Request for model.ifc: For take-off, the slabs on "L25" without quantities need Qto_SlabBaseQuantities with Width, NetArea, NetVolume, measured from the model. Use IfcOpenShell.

First a look at what the model holds.

```python
import ifcopenshell
import ifcopenshell.util.element
import ifcopenshell.util.unit

model = ifcopenshell.open("model.ifc")
print(model.schema)
for unit_type in ("LENGTHUNIT", "AREAUNIT", "VOLUMEUNIT"):
    print(unit_type, ifcopenshell.util.unit.calculate_unit_scale(model, unit_type))
storey = next(s for s in model.by_type("IfcBuildingStorey") if s.Name == "L25")
slabs = [e for e in ifcopenshell.util.element.get_decomposition(storey) if e.is_a("IfcSlab")]
for e in sorted(slabs, key=lambda e: e.id()):
    print(e.id(), e.is_a(), e.Name, list(ifcopenshell.util.element.get_psets(e, qtos_only=True)), sep=" | ")
```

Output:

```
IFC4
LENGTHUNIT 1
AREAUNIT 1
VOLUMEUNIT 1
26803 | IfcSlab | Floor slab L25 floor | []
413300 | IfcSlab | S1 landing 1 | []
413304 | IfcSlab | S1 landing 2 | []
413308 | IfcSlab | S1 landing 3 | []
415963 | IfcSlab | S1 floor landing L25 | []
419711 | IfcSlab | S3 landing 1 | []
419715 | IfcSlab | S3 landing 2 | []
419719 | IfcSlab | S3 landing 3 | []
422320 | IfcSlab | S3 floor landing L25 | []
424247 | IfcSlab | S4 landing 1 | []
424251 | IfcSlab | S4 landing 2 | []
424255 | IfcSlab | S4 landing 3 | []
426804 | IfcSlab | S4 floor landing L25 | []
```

```python
import ifcopenshell
import ifcopenshell.api.pset
import ifcopenshell.geom
import ifcopenshell.util.element
import ifcopenshell.util.shape
import ifcopenshell.util.unit

model = ifcopenshell.open("model.ifc")
unit_scale = ifcopenshell.util.unit.calculate_unit_scale(model)
area_scale = ifcopenshell.util.unit.calculate_unit_scale(model, "AREAUNIT")
volume_scale = ifcopenshell.util.unit.calculate_unit_scale(model, "VOLUMEUNIT")
settings = ifcopenshell.geom.settings()

storey = next(s for s in model.by_type("IfcBuildingStorey") if s.Name == "L25")
slabs = [e for e in ifcopenshell.util.element.get_decomposition(storey) if e.is_a("IfcSlab")]

for e in sorted(slabs, key=lambda e: e.id()):
    if ifcopenshell.util.element.get_psets(e, qtos_only=True, should_inherit=False):
        continue
    # Geometry comes back in metres, in the element's own axes.
    shape = ifcopenshell.geom.create_shape(settings, e)
    values = {
        "Width": ifcopenshell.util.shape.get_z(shape.geometry) / unit_scale,
        "NetArea": ifcopenshell.util.shape.get_footprint_area(shape.geometry) / area_scale,
        "NetVolume": ifcopenshell.util.shape.get_volume(shape.geometry) / volume_scale,
    }
    qto = ifcopenshell.api.pset.add_qto(model, product=e, name="Qto_SlabBaseQuantities")
    ifcopenshell.api.pset.edit_qto(model, qto=qto, properties=values)
    print(e.id(), {k: round(v, 3) for k, v in values.items()})

model.write("model-out.ifc")
```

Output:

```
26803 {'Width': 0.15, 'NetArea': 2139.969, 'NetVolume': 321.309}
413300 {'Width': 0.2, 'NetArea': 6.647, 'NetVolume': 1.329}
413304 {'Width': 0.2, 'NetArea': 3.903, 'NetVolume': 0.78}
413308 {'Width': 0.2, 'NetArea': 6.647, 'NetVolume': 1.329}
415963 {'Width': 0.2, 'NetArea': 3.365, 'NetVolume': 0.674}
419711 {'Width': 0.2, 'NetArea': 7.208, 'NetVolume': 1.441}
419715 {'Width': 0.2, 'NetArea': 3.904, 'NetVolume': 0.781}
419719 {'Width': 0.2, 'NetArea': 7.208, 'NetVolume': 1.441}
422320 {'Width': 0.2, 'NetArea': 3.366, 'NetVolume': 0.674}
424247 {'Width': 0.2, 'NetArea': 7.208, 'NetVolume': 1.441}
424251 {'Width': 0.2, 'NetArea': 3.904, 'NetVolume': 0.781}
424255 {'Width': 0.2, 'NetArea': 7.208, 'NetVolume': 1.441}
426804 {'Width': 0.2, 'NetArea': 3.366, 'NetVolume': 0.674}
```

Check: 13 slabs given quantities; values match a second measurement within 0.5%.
